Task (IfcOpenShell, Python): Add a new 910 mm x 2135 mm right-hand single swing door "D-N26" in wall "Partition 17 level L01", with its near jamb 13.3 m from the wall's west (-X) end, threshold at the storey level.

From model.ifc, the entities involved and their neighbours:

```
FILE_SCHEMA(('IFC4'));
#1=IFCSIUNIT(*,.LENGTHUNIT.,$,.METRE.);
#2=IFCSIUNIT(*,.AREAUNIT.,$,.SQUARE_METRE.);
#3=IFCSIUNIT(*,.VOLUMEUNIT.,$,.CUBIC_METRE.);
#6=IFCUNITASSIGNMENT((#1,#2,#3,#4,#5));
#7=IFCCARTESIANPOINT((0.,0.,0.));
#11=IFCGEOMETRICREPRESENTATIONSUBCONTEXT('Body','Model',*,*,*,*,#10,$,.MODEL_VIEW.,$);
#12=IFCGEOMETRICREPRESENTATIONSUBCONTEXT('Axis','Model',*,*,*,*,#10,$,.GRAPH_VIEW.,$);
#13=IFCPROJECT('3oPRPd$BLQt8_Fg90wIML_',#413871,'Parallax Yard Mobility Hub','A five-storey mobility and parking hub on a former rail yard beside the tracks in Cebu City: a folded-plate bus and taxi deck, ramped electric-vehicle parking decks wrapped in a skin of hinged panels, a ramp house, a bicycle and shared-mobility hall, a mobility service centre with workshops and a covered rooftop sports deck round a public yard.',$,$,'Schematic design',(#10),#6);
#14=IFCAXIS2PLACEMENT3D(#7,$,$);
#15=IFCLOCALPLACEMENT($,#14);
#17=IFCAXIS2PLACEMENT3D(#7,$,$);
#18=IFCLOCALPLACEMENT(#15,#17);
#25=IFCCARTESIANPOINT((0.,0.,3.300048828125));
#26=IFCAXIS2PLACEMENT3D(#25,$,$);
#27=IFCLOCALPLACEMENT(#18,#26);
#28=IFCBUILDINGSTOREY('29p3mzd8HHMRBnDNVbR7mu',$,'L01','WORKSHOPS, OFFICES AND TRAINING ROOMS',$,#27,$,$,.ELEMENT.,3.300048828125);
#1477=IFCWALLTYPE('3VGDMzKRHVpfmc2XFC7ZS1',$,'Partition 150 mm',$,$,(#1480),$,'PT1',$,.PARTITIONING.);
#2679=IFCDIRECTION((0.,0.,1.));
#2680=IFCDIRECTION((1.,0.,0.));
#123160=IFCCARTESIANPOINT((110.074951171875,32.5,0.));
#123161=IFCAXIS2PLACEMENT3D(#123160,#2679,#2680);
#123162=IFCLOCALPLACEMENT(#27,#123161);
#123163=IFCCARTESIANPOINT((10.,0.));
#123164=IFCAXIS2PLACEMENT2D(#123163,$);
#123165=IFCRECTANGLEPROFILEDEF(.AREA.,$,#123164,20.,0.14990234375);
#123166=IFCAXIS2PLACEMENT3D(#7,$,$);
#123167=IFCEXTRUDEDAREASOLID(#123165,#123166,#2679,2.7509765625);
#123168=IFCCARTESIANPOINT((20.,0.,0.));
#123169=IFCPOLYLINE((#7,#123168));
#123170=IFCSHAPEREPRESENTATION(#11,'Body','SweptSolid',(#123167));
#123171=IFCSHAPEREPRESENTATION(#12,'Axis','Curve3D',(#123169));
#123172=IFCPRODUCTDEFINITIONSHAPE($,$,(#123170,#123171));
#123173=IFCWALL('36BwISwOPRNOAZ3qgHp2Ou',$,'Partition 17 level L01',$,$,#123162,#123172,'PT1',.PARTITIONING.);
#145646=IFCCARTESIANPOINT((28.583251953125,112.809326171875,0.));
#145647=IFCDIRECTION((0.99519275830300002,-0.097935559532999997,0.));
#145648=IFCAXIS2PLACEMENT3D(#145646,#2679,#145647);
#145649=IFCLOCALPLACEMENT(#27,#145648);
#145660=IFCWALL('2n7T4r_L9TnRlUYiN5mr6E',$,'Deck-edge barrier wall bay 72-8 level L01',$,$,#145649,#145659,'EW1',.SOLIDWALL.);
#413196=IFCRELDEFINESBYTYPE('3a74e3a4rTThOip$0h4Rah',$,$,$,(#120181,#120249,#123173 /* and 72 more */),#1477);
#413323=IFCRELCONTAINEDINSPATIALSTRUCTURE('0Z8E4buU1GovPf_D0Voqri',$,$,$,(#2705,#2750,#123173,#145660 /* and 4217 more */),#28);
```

```python
import numpy as np
import ifcopenshell
import ifcopenshell.api.feature
import ifcopenshell.api.geometry
import ifcopenshell.api.root
import ifcopenshell.api.spatial
import ifcopenshell.geom
import ifcopenshell.util.element
import ifcopenshell.util.placement
import ifcopenshell.util.representation
import ifcopenshell.util.shape
import ifcopenshell.util.unit

model = ifcopenshell.open("model.ifc")
unit_scale = ifcopenshell.util.unit.calculate_unit_scale(model)
settings = ifcopenshell.geom.settings()


def volume(element):
    """Net volume in cubic metres, openings subtracted."""
    shape = ifcopenshell.geom.create_shape(settings, element)
    return ifcopenshell.util.shape.get_volume(shape.geometry)


wall = model.by_guid("36BwISwOPRNOAZ3qgHp2Ou")
storey = ifcopenshell.util.element.get_container(wall, ifc_class="IfcBuildingStorey")
context = ifcopenshell.util.representation.get_context(model, "Model", "Body", "MODEL_VIEW")
before = volume(wall)

width, height, from_end, sill = 0.91, 2.135, 13.3, 0.0  # metres

# The wall runs along its own X axis, and the end named is its -X end.
wall_shape = ifcopenshell.geom.create_shape(settings, wall)
x, y, z = ifcopenshell.util.shape.get_vertices(wall_shape.geometry).T
start = x.min() + from_end
face, thickness = float(y.min()), float(y.max() - y.min())
wall_matrix = ifcopenshell.util.placement.get_local_placement(wall.ObjectPlacement)
level = ifcopenshell.util.placement.get_local_placement(storey.ObjectPlacement)[2, 3]


def in_wall(x, y):
    """Placement at x, y metres in the wall's axes, at sill height."""
    matrix = wall_matrix.copy()
    matrix[:, 3] = wall_matrix @ np.array([x / unit_scale, y / unit_scale, 0.0, 1.0])
    matrix[2, 3] = level + sill / unit_scale
    return matrix


# Opening: a box that overshoots both wall faces by 50 mm.
opening = ifcopenshell.api.root.create_entity(model, ifc_class="IfcOpeningElement", predefined_type="OPENING")
box = ifcopenshell.api.geometry.add_wall_representation(
    model, context=context, length=width, height=height, thickness=thickness + 0.1
)
ifcopenshell.api.geometry.assign_representation(model, product=opening, representation=box)
ifcopenshell.api.geometry.edit_object_placement(model, product=opening, matrix=in_wall(start, face - 0.05), is_si=False)
ifcopenshell.api.feature.add_feature(model, feature=opening, element=wall)

door = ifcopenshell.api.root.create_entity(model, ifc_class="IfcDoor", name="D-N26", predefined_type="DOOR")
door.OverallWidth, door.OverallHeight = width / unit_scale, height / unit_scale
door.OperationType = "SINGLE_SWING_RIGHT"
body = ifcopenshell.api.geometry.add_door_representation(
    model,
    context=context,
    overall_width=door.OverallWidth,
    overall_height=door.OverallHeight,
    operation_type="SINGLE_SWING_RIGHT",
    lining_properties={"LiningDepth": thickness / unit_scale, "ThresholdDepth": thickness / unit_scale},
)
ifcopenshell.api.geometry.assign_representation(model, product=door, representation=body)
ifcopenshell.api.spatial.assign_container(model, products=[door], relating_structure=storey)
ifcopenshell.api.feature.add_filling(model, opening=opening, element=door)

# The lining spans the wall, so the door starts at the wall face.
ifcopenshell.api.geometry.edit_object_placement(model, product=door, matrix=in_wall(start, face), is_si=False)

after = volume(wall)

print(f"wall volume {before:.3f} -> {after:.3f} m3")

model.write("model_edited.ifc")
```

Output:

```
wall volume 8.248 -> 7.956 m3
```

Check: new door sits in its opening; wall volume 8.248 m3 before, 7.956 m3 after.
